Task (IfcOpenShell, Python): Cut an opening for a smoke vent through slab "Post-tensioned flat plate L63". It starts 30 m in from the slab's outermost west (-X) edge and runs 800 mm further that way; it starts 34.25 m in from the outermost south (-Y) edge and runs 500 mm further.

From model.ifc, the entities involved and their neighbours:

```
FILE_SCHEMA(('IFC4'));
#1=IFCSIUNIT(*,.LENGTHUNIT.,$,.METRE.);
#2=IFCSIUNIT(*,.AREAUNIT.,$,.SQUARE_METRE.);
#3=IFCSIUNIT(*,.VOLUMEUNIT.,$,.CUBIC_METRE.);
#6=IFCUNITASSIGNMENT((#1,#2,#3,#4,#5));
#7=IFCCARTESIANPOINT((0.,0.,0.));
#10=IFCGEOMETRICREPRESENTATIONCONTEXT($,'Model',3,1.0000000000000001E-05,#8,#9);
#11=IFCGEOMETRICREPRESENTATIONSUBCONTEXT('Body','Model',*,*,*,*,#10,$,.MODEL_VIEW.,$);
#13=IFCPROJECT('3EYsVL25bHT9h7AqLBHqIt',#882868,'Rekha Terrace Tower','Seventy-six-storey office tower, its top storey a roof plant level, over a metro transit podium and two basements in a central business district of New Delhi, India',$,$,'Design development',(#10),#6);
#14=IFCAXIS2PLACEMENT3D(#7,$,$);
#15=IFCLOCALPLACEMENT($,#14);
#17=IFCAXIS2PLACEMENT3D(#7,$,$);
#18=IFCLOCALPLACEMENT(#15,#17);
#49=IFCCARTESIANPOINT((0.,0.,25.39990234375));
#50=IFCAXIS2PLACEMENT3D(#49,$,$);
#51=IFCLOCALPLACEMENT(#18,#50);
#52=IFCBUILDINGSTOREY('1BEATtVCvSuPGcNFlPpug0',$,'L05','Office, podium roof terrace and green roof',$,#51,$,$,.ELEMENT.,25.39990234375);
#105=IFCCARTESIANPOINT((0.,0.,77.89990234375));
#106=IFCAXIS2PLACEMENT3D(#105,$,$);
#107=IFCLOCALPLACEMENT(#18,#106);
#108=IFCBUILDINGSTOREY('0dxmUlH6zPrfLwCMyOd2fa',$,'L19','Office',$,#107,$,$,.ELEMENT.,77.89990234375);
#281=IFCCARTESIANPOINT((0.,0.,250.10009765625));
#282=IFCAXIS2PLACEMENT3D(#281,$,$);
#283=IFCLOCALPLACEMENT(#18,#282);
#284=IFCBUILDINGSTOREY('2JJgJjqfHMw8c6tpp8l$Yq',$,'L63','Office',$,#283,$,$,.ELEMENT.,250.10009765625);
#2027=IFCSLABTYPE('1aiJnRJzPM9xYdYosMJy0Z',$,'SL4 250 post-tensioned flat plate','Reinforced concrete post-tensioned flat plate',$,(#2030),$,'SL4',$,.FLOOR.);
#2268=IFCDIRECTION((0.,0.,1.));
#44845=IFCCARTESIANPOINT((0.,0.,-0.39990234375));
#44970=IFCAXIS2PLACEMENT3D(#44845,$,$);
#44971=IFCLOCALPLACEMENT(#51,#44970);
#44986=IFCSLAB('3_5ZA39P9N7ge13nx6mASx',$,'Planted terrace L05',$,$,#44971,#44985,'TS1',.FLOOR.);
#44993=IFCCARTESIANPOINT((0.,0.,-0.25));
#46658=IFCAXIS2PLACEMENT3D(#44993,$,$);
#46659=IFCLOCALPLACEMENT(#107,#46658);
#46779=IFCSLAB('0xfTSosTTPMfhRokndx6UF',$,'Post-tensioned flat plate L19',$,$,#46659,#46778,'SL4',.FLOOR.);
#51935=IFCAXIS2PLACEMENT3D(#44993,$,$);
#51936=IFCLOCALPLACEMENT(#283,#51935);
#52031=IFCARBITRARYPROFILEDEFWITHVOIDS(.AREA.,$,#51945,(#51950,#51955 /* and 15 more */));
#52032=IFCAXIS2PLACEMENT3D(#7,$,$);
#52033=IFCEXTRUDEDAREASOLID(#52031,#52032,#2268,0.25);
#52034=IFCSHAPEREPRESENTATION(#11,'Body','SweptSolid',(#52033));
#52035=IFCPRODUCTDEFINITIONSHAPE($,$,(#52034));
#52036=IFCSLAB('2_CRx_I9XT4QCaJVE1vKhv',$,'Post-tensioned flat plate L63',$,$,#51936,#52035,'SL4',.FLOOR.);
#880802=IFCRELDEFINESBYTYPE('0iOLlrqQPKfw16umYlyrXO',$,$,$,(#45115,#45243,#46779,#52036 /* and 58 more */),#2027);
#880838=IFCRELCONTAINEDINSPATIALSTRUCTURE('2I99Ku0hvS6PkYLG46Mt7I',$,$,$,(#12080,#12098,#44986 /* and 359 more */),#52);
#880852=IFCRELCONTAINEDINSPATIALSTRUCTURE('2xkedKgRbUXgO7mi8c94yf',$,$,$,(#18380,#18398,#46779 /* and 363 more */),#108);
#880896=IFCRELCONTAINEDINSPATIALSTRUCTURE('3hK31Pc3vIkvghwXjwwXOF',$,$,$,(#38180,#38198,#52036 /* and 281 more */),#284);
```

```python
import numpy as np
import ifcopenshell
import ifcopenshell.api.feature
import ifcopenshell.api.geometry
import ifcopenshell.api.root
import ifcopenshell.geom
import ifcopenshell.util.placement
import ifcopenshell.util.representation
import ifcopenshell.util.shape
import ifcopenshell.util.unit

model = ifcopenshell.open("model.ifc")
unit_scale = ifcopenshell.util.unit.calculate_unit_scale(model)
settings = ifcopenshell.geom.settings()


def volume(element):
    """Net volume in cubic metres, openings subtracted."""
    shape = ifcopenshell.geom.create_shape(settings, element)
    return ifcopenshell.util.shape.get_volume(shape.geometry)


slab = model.by_guid("2_CRx_I9XT4QCaJVE1vKhv")
before = volume(slab)

# Extent in the slab's own axes, in metres. The edges named are its -X and -Y sides.
slab_shape = ifcopenshell.geom.create_shape(settings, slab)
vertices = ifcopenshell.util.shape.get_vertices(slab_shape.geometry)
x_min, y_min, bottom = vertices.min(axis=0)
top = vertices[:, 2].max()

opening = ifcopenshell.api.root.create_entity(model, ifc_class="IfcOpeningElement", name="Smoke vent opening", predefined_type="OPENING")
context = ifcopenshell.util.representation.get_context(model, "Model", "Body", "MODEL_VIEW")
width, depth = 0.8, 0.5
outline = [(0.0, 0.0), (width, 0.0), (width, depth), (0.0, depth), (0.0, 0.0)]
# Overshoot both faces by 50 mm so the cut is clean.
shape = ifcopenshell.api.geometry.add_slab_representation(
    model, context=context, depth=top - bottom + 0.1, polyline=outline
)
ifcopenshell.api.geometry.assign_representation(model, product=opening, representation=shape)

matrix = ifcopenshell.util.placement.get_local_placement(slab.ObjectPlacement)
matrix[:, 3] = matrix @ np.append(np.array([x_min + 30, y_min + 34.25, bottom - 0.05]) / unit_scale, 1.0)
ifcopenshell.api.geometry.edit_object_placement(model, product=opening, matrix=matrix, is_si=False)
ifcopenshell.api.feature.add_feature(model, feature=opening, element=slab)

after = volume(slab)

print(f"slab volume {before:.3f} -> {after:.3f} m3")

model.write("model_edited.ifc")
```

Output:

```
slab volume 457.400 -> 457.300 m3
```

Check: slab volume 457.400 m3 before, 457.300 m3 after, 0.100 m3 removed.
